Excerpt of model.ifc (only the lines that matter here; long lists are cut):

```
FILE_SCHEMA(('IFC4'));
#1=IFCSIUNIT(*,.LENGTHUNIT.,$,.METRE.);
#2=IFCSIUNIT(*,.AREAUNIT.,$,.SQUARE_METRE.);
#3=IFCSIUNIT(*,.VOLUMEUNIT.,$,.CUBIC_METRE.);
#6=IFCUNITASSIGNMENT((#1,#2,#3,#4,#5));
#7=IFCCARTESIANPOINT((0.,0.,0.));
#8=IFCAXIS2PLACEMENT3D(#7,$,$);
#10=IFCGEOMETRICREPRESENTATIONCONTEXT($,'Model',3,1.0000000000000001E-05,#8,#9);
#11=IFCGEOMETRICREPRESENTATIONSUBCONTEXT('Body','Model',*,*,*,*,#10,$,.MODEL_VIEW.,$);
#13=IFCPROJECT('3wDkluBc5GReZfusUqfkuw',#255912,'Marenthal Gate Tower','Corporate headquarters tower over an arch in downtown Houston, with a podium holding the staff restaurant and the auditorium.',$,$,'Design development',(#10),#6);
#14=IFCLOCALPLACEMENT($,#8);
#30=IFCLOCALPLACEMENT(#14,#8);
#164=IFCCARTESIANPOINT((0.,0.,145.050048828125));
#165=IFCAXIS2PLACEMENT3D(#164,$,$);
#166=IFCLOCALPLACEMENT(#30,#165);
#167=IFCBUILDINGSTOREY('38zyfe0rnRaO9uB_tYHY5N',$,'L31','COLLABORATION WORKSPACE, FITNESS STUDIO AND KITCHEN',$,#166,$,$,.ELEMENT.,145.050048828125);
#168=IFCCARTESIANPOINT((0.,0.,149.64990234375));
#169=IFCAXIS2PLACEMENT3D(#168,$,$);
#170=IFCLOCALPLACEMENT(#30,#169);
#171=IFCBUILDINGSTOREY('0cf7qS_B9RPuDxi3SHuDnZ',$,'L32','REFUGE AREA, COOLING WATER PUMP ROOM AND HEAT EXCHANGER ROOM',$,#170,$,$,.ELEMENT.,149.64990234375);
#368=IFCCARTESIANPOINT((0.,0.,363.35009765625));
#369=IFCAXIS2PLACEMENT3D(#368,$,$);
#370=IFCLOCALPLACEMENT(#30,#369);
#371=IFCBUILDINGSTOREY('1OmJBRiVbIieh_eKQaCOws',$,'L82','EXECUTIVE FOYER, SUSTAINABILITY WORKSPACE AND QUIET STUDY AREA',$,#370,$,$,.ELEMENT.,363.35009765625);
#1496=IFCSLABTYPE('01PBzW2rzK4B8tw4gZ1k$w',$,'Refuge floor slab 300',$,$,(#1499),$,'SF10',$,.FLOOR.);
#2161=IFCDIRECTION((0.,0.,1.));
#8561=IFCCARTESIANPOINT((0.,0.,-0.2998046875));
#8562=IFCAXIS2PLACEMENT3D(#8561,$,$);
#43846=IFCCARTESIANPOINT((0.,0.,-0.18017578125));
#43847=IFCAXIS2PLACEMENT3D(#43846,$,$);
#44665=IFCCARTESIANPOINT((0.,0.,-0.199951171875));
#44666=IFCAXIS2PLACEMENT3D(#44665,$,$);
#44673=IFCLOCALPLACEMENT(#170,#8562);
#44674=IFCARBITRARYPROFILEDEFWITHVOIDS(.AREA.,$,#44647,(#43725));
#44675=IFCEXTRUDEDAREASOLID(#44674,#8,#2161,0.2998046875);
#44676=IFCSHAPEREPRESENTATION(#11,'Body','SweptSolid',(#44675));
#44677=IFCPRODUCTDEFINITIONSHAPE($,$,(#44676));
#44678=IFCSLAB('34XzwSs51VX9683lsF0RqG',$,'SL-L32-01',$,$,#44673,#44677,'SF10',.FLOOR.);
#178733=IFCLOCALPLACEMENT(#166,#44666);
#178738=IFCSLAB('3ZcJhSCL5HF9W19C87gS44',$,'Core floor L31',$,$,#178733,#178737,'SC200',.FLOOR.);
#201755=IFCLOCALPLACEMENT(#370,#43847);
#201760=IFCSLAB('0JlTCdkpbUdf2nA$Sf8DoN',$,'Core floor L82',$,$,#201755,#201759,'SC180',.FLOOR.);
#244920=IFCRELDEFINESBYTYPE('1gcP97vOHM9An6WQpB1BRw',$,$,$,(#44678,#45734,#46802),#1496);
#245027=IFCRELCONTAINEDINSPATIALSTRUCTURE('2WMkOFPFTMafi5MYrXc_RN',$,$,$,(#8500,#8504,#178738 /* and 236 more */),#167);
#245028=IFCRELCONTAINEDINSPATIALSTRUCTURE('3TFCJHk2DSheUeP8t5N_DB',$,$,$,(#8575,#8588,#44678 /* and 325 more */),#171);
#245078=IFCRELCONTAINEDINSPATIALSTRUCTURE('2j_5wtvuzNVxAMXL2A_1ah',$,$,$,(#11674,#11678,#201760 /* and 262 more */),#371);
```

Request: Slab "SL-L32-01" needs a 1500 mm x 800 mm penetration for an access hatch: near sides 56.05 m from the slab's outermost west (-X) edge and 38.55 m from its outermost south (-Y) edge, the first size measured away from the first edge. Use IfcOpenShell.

```python
import numpy as np
import ifcopenshell
import ifcopenshell.api.feature
import ifcopenshell.api.geometry
import ifcopenshell.api.root
import ifcopenshell.geom
import ifcopenshell.util.placement
import ifcopenshell.util.representation
import ifcopenshell.util.shape
import ifcopenshell.util.unit

model = ifcopenshell.open("model.ifc")
unit_scale = ifcopenshell.util.unit.calculate_unit_scale(model)
settings = ifcopenshell.geom.settings()


def volume(element):
    """Net volume in cubic metres, openings subtracted."""
    shape = ifcopenshell.geom.create_shape(settings, element)
    return ifcopenshell.util.shape.get_volume(shape.geometry)


slab = model.by_guid("34XzwSs51VX9683lsF0RqG")
before = volume(slab)

# Extent in the slab's own axes, in metres. The edges named are its -X and -Y sides.
slab_shape = ifcopenshell.geom.create_shape(settings, slab)
vertices = ifcopenshell.util.shape.get_vertices(slab_shape.geometry)
x_min, y_min, bottom = vertices.min(axis=0)
top = vertices[:, 2].max()

opening = ifcopenshell.api.root.create_entity(model, ifc_class="IfcOpeningElement", name="Access hatch opening", predefined_type="OPENING")
context = ifcopenshell.util.representation.get_context(model, "Model", "Body", "MODEL_VIEW")
width, depth = 1.5, 0.8
outline = [(0.0, 0.0), (width, 0.0), (width, depth), (0.0, depth), (0.0, 0.0)]
# Overshoot both faces by 50 mm so the cut is clean.
shape = ifcopenshell.api.geometry.add_slab_representation(
    model, context=context, depth=top - bottom + 0.1, polyline=outline
)
ifcopenshell.api.geometry.assign_representation(model, product=opening, representation=shape)

matrix = ifcopenshell.util.placement.get_local_placement(slab.ObjectPlacement)
matrix[:, 3] = matrix @ np.append(np.array([x_min + 56.05, y_min + 38.55, bottom - 0.05]) / unit_scale, 1.0)
ifcopenshell.api.geometry.edit_object_placement(model, product=opening, matrix=matrix, is_si=False)
ifcopenshell.api.feature.add_feature(model, feature=opening, element=slab)

after = volume(slab)

print(f"slab volume {before:.3f} -> {after:.3f} m3")

model.write("model_v2.ifc")
```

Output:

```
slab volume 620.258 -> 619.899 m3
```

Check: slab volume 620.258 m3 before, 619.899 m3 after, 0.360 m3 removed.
